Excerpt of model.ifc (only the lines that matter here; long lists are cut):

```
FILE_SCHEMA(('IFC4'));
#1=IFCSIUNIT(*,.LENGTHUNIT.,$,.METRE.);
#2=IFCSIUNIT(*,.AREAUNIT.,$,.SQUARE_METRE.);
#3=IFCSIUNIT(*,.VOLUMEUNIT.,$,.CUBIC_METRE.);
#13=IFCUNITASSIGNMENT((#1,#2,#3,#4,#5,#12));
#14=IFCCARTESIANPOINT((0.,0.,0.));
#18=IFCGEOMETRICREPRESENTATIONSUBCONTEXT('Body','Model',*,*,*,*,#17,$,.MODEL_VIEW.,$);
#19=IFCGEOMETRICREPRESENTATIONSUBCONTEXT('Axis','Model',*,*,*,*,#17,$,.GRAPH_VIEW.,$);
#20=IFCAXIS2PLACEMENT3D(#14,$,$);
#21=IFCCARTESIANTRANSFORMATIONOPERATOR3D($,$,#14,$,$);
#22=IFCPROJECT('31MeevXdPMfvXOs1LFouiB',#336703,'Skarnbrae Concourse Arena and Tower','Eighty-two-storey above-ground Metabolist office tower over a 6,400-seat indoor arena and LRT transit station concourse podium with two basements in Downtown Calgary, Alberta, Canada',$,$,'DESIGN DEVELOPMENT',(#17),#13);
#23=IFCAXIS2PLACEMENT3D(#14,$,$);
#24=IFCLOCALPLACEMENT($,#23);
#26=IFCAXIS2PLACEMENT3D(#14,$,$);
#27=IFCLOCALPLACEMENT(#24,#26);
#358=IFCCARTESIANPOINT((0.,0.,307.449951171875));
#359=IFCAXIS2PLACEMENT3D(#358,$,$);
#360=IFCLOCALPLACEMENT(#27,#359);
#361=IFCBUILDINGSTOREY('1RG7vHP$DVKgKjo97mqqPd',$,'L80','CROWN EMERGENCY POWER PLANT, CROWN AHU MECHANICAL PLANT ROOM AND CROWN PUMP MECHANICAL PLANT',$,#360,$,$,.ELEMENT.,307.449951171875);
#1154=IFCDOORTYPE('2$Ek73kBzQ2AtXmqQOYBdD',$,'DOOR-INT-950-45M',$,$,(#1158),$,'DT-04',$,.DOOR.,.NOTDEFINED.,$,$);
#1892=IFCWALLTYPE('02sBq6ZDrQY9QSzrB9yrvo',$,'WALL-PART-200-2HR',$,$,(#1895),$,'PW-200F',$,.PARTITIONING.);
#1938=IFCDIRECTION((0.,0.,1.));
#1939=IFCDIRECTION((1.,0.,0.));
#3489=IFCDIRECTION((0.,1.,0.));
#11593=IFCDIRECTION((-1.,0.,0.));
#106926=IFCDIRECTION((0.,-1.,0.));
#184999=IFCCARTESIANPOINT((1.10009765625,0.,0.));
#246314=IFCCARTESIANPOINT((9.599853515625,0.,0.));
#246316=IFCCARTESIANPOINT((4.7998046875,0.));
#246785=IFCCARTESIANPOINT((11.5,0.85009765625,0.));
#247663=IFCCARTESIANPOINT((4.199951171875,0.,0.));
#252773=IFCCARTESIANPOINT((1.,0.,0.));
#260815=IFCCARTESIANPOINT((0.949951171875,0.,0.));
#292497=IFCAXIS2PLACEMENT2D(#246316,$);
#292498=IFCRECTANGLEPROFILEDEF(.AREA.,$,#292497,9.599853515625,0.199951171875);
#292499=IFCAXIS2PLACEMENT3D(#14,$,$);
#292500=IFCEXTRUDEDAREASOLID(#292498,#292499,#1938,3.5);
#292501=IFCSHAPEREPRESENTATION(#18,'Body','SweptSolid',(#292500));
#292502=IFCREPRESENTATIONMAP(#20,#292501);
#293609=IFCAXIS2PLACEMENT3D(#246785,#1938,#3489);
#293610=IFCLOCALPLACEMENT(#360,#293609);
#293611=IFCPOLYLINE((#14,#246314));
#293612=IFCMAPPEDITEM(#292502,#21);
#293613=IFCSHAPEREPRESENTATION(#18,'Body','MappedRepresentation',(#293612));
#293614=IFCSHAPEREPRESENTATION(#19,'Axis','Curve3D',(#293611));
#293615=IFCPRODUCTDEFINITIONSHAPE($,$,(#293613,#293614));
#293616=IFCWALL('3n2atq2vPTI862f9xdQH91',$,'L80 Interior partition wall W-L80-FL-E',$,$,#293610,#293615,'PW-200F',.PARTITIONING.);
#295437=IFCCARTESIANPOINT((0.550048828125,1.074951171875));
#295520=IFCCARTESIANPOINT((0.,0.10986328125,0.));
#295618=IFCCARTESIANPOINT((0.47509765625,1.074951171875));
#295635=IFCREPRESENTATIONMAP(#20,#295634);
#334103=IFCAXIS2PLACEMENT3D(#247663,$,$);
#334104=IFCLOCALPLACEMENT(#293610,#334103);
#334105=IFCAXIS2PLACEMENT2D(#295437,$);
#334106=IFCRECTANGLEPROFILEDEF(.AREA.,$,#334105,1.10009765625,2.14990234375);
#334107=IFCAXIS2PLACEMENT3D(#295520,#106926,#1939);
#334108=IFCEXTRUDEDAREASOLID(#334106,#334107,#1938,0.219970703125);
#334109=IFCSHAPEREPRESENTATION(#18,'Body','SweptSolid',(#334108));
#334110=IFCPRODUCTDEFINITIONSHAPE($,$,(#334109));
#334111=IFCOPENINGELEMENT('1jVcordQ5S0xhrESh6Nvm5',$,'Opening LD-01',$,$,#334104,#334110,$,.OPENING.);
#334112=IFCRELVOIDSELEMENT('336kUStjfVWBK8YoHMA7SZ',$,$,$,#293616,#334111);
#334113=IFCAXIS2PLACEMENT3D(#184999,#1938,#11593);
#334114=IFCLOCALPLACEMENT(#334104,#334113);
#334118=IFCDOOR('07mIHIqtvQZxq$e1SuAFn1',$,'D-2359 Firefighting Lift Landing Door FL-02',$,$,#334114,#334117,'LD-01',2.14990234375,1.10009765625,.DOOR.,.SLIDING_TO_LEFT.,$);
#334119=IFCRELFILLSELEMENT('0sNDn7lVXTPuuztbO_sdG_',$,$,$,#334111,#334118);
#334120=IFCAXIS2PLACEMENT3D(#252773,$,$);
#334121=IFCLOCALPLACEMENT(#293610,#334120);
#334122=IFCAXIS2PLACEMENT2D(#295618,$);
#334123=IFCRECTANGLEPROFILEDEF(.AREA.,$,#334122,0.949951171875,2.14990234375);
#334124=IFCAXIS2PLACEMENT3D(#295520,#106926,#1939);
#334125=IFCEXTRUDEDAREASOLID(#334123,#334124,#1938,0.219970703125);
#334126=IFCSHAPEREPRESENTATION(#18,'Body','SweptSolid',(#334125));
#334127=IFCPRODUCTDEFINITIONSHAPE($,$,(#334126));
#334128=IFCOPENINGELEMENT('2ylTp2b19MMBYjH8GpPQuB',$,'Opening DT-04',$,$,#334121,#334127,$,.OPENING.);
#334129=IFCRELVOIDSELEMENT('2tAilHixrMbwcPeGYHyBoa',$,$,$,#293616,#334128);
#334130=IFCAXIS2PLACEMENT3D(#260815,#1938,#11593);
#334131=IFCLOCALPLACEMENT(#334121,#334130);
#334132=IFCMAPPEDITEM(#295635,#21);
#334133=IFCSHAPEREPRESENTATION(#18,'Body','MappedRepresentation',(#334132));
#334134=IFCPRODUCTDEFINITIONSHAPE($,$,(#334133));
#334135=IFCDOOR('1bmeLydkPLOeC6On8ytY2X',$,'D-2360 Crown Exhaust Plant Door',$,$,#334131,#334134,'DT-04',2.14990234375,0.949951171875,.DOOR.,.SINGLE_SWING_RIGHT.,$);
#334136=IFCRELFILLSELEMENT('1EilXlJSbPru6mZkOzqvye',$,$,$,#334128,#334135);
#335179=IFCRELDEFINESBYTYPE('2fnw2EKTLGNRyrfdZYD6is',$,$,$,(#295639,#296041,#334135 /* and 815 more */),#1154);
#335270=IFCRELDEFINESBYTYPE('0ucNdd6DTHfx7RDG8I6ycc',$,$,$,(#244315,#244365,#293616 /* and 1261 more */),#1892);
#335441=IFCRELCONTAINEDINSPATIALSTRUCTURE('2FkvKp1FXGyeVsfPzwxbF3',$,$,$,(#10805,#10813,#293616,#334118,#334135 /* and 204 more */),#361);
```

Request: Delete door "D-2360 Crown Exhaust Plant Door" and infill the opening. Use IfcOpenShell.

```python
import ifcopenshell
import ifcopenshell.api.feature
import ifcopenshell.api.root
import ifcopenshell.geom
import ifcopenshell.util.shape

model = ifcopenshell.open("model.ifc")
settings = ifcopenshell.geom.settings()


def volume(element):
    """Net volume in cubic metres, openings subtracted."""
    shape = ifcopenshell.geom.create_shape(settings, element)
    return ifcopenshell.util.shape.get_volume(shape.geometry)


door = model.by_guid("1bmeLydkPLOeC6On8ytY2X")
opening = door.FillsVoids[0].RelatingOpeningElement
wall = opening.VoidsElements[0].RelatingBuildingElement
before = volume(wall)

ifcopenshell.api.root.remove_product(model, product=door)
ifcopenshell.api.feature.remove_feature(model, feature=opening)

after = volume(wall)

print(f"wall volume {before:.3f} -> {after:.3f} m3")

model.write("model-out.ifc")
```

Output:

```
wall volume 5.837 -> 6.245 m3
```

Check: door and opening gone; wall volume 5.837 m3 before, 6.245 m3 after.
